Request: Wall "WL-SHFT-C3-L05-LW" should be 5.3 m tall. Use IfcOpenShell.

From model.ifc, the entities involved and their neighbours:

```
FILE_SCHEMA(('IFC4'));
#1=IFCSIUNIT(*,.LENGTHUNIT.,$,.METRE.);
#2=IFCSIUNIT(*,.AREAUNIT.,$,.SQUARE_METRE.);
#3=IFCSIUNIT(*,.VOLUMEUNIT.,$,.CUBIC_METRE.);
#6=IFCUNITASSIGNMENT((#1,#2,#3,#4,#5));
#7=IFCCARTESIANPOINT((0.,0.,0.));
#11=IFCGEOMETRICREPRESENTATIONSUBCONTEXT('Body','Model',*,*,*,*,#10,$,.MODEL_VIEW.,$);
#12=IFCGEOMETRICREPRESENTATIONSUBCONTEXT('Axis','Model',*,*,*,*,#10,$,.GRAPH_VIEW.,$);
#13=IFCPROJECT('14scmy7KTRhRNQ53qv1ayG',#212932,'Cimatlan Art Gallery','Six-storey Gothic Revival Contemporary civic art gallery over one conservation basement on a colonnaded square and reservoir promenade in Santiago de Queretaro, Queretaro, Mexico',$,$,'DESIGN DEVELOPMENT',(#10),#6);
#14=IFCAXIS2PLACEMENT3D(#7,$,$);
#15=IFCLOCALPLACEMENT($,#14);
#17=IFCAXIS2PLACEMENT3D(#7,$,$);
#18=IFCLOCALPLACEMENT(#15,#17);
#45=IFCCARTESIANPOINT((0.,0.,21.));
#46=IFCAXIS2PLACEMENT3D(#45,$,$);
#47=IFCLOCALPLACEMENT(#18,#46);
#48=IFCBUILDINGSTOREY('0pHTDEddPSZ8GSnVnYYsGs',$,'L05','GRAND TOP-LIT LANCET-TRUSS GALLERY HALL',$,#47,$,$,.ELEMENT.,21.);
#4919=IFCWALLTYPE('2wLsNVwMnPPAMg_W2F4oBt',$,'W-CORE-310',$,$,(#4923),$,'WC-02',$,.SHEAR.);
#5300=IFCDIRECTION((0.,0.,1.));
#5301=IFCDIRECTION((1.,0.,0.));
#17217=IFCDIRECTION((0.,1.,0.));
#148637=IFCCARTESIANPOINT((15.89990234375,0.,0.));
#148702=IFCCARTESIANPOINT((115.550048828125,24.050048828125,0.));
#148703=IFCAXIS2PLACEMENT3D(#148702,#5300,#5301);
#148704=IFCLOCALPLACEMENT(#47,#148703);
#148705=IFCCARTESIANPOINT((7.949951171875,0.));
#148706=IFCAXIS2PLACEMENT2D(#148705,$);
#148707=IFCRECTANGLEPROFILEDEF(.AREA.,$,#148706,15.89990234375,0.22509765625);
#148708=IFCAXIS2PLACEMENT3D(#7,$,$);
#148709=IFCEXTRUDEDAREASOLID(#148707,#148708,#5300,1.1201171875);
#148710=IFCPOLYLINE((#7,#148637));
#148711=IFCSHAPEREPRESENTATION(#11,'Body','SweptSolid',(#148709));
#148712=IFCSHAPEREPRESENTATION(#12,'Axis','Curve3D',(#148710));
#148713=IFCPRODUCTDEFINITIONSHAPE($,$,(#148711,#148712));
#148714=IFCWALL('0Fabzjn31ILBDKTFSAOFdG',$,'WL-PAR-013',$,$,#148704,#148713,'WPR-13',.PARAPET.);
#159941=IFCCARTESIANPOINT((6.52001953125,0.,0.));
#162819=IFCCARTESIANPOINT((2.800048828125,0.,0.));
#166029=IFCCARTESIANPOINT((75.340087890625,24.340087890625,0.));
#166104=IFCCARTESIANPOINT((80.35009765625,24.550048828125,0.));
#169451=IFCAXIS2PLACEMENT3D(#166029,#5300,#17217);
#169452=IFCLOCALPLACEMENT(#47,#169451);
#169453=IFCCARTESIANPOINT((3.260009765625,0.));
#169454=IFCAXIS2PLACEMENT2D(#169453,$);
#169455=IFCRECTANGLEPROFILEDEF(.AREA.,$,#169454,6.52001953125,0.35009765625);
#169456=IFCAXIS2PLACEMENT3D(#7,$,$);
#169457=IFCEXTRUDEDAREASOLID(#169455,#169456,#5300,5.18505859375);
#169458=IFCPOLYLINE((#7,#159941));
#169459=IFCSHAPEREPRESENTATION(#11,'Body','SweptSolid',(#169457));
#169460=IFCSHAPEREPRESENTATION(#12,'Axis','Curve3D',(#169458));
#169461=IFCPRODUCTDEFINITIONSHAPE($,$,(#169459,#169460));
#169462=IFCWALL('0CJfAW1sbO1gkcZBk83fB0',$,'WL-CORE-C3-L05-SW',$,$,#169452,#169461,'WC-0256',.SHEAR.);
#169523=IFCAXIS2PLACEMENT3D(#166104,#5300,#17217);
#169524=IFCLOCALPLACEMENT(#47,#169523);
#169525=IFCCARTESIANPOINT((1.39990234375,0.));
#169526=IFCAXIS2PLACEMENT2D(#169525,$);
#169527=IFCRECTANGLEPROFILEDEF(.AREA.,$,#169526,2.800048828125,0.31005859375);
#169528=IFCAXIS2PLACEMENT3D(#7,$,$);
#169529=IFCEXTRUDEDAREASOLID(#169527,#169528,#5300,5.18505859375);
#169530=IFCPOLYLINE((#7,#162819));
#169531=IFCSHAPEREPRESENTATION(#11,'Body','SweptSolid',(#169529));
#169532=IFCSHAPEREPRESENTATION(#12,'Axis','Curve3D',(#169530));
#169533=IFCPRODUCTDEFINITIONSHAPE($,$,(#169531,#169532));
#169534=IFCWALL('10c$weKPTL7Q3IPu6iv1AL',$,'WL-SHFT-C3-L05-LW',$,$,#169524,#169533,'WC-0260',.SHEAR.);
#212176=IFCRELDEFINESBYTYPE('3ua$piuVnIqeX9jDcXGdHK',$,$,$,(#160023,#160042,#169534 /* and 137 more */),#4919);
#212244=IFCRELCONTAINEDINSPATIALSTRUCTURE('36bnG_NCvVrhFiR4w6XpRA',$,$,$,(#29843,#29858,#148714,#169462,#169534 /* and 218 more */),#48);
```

```python
import ifcopenshell
import ifcopenshell.geom
import ifcopenshell.util.representation
import ifcopenshell.util.shape
import ifcopenshell.util.unit

model = ifcopenshell.open("model.ifc")
unit_scale = ifcopenshell.util.unit.calculate_unit_scale(model)
settings = ifcopenshell.geom.settings()


def volume(element):
    """Net volume in cubic metres, openings subtracted."""
    shape = ifcopenshell.geom.create_shape(settings, element)
    return ifcopenshell.util.shape.get_volume(shape.geometry)


wall = model.by_guid("10c$weKPTL7Q3IPu6iv1AL")
before = volume(wall)

body = ifcopenshell.util.representation.get_representation(wall, "Model", "Body")
solid = body.Items[0]
old_height = solid.Depth
solid.Depth = 5.3 / unit_scale
after = volume(wall)

print(f"height {old_height:g} -> {solid.Depth:g}, volume {before:.3f} -> {after:.3f} m3")

model.write("model_updated.ifc")
```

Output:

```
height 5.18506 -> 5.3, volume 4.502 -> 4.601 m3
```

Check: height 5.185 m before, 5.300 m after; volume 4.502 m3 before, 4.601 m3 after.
